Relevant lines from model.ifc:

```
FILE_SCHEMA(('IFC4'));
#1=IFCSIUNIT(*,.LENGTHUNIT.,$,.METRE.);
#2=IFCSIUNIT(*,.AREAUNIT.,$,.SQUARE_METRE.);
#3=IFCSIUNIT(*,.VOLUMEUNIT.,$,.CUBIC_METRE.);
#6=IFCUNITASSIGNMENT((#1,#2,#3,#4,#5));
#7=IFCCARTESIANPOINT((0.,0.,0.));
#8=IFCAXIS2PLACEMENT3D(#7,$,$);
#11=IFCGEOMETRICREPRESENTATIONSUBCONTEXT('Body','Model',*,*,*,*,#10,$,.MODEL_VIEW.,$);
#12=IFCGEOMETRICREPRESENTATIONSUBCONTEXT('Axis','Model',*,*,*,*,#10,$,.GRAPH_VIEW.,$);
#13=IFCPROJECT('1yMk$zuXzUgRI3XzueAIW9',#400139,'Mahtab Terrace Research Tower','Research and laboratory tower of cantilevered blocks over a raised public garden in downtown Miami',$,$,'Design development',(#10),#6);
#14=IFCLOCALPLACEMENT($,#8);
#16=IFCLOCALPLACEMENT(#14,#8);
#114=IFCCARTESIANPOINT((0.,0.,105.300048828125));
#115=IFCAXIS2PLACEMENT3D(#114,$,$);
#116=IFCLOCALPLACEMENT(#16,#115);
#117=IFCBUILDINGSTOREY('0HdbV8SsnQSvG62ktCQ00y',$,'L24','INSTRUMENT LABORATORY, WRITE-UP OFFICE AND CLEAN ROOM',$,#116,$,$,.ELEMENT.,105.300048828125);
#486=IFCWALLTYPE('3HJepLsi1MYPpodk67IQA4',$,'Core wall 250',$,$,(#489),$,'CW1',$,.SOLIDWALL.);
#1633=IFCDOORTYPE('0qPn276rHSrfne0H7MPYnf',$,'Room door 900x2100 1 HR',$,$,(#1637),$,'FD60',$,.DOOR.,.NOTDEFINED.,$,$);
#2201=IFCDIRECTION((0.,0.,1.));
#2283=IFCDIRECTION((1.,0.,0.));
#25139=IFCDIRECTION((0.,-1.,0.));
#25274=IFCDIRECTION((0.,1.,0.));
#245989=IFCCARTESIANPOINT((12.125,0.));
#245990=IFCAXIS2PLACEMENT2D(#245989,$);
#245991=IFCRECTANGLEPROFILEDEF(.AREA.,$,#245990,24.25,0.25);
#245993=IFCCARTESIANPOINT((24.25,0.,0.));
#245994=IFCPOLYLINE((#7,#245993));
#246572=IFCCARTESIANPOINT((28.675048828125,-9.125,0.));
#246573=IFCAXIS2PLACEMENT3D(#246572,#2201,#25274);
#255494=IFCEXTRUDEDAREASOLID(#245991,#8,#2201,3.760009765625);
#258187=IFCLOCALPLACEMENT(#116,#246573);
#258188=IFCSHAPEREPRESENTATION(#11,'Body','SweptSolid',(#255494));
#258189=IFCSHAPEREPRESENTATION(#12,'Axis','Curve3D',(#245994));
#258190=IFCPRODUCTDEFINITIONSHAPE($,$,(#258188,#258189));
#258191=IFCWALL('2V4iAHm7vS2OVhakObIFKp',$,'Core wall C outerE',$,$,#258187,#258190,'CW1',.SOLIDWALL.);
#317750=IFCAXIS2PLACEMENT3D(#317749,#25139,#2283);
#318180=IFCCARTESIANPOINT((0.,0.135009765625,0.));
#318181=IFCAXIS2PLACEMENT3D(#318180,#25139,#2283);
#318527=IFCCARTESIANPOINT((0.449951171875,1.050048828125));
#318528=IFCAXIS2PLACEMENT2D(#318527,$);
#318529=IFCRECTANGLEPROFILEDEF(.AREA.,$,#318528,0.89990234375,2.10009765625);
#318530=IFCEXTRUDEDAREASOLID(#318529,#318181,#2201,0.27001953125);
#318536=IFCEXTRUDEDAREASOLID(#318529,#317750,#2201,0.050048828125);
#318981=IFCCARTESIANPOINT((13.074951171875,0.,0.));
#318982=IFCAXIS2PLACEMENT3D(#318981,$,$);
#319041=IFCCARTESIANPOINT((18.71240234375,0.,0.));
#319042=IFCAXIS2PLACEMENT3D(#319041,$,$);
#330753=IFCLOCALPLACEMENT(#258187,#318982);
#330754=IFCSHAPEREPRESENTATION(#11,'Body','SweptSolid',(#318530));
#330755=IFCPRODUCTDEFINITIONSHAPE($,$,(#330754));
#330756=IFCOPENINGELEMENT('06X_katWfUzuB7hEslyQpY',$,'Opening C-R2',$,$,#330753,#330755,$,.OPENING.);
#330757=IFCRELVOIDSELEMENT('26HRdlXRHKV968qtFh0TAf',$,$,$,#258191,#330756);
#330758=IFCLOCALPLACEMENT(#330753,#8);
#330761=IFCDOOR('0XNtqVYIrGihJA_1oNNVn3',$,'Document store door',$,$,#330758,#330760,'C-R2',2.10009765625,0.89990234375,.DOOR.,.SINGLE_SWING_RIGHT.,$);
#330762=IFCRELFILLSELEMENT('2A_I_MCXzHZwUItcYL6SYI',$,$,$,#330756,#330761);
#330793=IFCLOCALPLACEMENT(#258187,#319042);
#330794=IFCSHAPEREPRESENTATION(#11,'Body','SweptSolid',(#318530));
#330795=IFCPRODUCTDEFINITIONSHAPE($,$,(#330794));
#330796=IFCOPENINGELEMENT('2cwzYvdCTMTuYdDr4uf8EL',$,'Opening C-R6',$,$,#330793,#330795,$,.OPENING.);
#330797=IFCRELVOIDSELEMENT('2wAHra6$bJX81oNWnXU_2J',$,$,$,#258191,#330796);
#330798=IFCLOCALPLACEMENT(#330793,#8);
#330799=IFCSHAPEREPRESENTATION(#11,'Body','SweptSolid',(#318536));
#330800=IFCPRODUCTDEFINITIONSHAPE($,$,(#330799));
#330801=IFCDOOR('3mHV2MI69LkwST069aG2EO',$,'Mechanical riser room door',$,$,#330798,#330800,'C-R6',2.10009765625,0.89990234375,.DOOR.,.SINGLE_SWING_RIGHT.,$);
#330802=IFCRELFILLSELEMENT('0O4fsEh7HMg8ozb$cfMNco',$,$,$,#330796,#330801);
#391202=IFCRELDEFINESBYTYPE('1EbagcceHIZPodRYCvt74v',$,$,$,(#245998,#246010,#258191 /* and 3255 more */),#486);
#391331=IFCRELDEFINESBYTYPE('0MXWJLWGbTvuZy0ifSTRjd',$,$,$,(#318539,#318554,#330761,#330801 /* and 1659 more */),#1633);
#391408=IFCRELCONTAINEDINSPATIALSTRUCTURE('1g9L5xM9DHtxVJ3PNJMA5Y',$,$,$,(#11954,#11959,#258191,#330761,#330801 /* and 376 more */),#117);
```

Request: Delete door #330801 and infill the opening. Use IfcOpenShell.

```python
import ifcopenshell
import ifcopenshell.api.feature
import ifcopenshell.api.root
import ifcopenshell.geom
import ifcopenshell.util.shape

model = ifcopenshell.open("model.ifc")
settings = ifcopenshell.geom.settings()


def volume(element):
    """Net volume in cubic metres, openings subtracted."""
    shape = ifcopenshell.geom.create_shape(settings, element)
    return ifcopenshell.util.shape.get_volume(shape.geometry)


door = model.by_guid("3mHV2MI69LkwST069aG2EO")
opening = door.FillsVoids[0].RelatingOpeningElement
wall = opening.VoidsElements[0].RelatingBuildingElement
before = volume(wall)

ifcopenshell.api.root.remove_product(model, product=door)
ifcopenshell.api.feature.remove_feature(model, feature=opening)

after = volume(wall)

print(f"wall volume {before:.3f} -> {after:.3f} m3")

model.write("model_edited.ifc")
```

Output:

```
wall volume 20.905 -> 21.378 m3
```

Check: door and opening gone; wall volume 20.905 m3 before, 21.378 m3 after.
